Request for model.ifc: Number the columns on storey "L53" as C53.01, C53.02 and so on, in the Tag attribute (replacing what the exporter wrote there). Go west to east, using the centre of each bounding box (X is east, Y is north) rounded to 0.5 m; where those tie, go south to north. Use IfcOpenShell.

First a look at what the model holds.

```python
import ifcopenshell
import ifcopenshell.util.element
import ifcopenshell.util.placement

model = ifcopenshell.open("model.ifc")
print(model.schema)
storey = next(s for s in model.by_type("IfcBuildingStorey") if s.Name == "L53")
columns = [e for e in ifcopenshell.util.element.get_decomposition(storey) if e.is_a("IfcColumn")]
for e in sorted(columns, key=lambda e: e.id()):
    origin = ifcopenshell.util.placement.get_local_placement(e.ObjectPlacement)[:3, 3]
    print(e.id(), e.Tag, e.Name, origin.round(2) + 0.0, sep=" | ")
```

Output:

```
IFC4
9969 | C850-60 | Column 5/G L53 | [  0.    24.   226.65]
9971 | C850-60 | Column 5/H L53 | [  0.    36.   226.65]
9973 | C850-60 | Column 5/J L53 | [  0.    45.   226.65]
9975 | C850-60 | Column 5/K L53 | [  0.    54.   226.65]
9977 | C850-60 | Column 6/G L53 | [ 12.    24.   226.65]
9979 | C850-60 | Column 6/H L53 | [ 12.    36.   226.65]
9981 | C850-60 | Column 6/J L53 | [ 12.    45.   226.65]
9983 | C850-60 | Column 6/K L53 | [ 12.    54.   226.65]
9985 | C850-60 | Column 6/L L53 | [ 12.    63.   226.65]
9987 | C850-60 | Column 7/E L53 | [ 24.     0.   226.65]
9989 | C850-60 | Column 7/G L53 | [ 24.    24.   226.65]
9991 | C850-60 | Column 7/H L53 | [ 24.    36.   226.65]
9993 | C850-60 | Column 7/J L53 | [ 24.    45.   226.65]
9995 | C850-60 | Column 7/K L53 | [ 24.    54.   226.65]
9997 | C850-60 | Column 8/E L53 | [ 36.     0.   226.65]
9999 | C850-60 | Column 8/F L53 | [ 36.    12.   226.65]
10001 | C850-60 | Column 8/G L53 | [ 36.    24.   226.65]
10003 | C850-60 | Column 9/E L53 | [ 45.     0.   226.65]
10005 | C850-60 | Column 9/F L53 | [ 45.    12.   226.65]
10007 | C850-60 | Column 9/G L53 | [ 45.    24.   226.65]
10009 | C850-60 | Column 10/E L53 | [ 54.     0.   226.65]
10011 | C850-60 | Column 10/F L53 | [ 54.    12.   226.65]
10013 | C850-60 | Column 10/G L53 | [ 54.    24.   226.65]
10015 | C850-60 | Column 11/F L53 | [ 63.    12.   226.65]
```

```python
import ifcopenshell
import ifcopenshell.geom
import ifcopenshell.util.element
import ifcopenshell.util.shape

model = ifcopenshell.open("model.ifc")
settings = ifcopenshell.geom.settings()
settings.set("use-world-coords", True)


def centre(element):
    shape = ifcopenshell.geom.create_shape(settings, element)
    return ifcopenshell.util.shape.get_bbox_centroid(shape.geometry)


storey = next(s for s in model.by_type("IfcBuildingStorey") if s.Name == "L53")
columns = [e for e in ifcopenshell.util.element.get_decomposition(storey) if e.is_a("IfcColumn")]

# Insertion points can sit at a corner or the storey origin, so sort by the geometry (in metres).
centres = {e: centre(e) for e in columns}
columns.sort(key=lambda e: (round(centres[e][0] / 0.5), centres[e][1]))

for i, e in enumerate(columns, start=1):
    number = f"C53.{i:02d}"
    e.Tag = number
    print(e.id(), number)

model.write("model_rev.ifc")
```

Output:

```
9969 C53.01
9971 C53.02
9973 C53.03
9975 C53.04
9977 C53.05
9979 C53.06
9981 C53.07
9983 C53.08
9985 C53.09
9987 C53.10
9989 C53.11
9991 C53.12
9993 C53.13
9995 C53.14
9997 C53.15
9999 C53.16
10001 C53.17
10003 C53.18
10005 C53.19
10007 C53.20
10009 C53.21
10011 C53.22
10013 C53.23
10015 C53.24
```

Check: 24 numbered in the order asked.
